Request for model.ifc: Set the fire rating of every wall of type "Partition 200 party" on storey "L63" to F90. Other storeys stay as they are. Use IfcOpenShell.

First a look at what the model holds.

```python
import ifcopenshell
import ifcopenshell.util.element

model = ifcopenshell.open("model.ifc")
print(model.schema)
storey = next(s for s in model.by_type("IfcBuildingStorey") if s.Name == "L63")
walls = [e for e in ifcopenshell.util.element.get_decomposition(storey) if e.is_a("IfcWall")]
seen = {}
for e in walls:
    element_type = ifcopenshell.util.element.get_type(e)
    key = (element_type.Name if element_type != e and element_type else None, ifcopenshell.util.element.get_pset(e, "Pset_WallCommon", "FireRating"))
    seen[key] = seen.get(key, 0) + 1
for (name, value), count in sorted(seen.items(), key=str):
    print(count, "x", name, "|", value)
```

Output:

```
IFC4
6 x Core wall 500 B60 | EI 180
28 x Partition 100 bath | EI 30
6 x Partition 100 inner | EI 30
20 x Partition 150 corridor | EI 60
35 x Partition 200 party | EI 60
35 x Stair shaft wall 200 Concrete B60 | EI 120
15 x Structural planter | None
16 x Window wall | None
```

```python
import ifcopenshell
import ifcopenshell.api.pset
import ifcopenshell.util.element

model = ifcopenshell.open("model.ifc")

storey = next(s for s in model.by_type("IfcBuildingStorey") if s.Name == "L63")
walls = [e for e in ifcopenshell.util.element.get_decomposition(storey) if e.is_a("IfcWall")]

count = 0
for e in walls:
    element_type = ifcopenshell.util.element.get_type(e)
    if element_type in (None, e) or element_type.Name != "Partition 200 party":
        continue
    found = ifcopenshell.util.element.get_pset(e, "Pset_WallCommon", should_inherit=False)
    if found:
        pset = model.by_id(found["id"])
        if len(ifcopenshell.util.element.get_elements_by_pset(pset)) > 1:
            pset = ifcopenshell.api.pset.unshare_pset(model, products=[e], pset=pset)[0]
    else:
        pset = ifcopenshell.api.pset.add_pset(model, product=e, name="Pset_WallCommon")
    ifcopenshell.api.pset.edit_pset(model, pset=pset, properties={"FireRating": "F90"})
    count += 1

print(count, "walls updated")

model.write("model_updated.ifc")
```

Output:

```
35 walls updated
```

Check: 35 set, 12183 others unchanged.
